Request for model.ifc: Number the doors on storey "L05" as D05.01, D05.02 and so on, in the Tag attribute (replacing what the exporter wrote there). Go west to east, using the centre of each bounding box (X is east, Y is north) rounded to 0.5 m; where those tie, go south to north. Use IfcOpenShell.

First a look at what the model holds.

```python
import ifcopenshell
import ifcopenshell.util.element
import ifcopenshell.util.placement

model = ifcopenshell.open("model.ifc")
print(model.schema)
storey = next(s for s in model.by_type("IfcBuildingStorey") if s.Name == "L05")
doors = [e for e in ifcopenshell.util.element.get_decomposition(storey) if e.is_a("IfcDoor")]
for e in sorted(doors, key=lambda e: e.id()):
    origin = ifcopenshell.util.placement.get_local_placement(e.ObjectPlacement)[:3, 3]
    print(e.id(), e.Tag, e.Name, origin.round(2) + 0.0, sep=" | ")
```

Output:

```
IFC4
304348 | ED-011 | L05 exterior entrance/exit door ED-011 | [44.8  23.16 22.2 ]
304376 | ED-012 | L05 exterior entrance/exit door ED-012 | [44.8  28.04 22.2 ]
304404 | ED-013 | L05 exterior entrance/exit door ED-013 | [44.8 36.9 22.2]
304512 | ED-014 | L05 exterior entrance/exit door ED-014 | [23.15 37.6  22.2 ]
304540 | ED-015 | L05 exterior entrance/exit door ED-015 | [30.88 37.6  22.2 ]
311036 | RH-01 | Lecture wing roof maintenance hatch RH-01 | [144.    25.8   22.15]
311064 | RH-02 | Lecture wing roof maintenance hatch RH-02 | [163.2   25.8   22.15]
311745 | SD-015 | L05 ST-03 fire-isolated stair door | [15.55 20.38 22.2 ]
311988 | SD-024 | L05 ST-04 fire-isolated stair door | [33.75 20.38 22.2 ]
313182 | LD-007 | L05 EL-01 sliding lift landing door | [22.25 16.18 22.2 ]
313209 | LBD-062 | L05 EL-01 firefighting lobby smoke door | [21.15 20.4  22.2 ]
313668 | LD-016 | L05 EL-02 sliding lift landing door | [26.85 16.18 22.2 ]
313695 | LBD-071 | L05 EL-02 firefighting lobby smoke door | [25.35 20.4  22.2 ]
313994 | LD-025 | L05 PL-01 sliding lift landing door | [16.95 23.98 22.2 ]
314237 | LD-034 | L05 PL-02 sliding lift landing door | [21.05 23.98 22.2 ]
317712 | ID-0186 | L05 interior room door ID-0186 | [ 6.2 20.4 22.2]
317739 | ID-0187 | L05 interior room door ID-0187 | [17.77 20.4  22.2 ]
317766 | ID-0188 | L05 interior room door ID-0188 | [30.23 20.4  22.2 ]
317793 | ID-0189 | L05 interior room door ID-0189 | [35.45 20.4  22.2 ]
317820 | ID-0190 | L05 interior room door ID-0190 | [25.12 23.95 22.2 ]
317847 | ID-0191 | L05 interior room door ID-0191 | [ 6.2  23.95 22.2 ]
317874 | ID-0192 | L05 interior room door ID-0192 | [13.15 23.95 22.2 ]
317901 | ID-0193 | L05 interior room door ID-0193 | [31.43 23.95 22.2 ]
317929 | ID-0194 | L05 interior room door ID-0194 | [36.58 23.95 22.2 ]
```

```python
import ifcopenshell
import ifcopenshell.geom
import ifcopenshell.util.element
import ifcopenshell.util.shape

model = ifcopenshell.open("model.ifc")
settings = ifcopenshell.geom.settings()
settings.set("use-world-coords", True)


def centre(element):
    shape = ifcopenshell.geom.create_shape(settings, element)
    return ifcopenshell.util.shape.get_bbox_centroid(shape.geometry)


storey = next(s for s in model.by_type("IfcBuildingStorey") if s.Name == "L05")
doors = [e for e in ifcopenshell.util.element.get_decomposition(storey) if e.is_a("IfcDoor")]

# Insertion points can sit at a corner or the storey origin, so sort by the geometry (in metres).
centres = {e: centre(e) for e in doors}
doors.sort(key=lambda e: (round(centres[e][0] / 0.5), centres[e][1]))

for i, e in enumerate(doors, start=1):
    number = f"D05.{i:02d}"
    e.Tag = number
    print(e.id(), number)

model.write("model_v2.ifc")
```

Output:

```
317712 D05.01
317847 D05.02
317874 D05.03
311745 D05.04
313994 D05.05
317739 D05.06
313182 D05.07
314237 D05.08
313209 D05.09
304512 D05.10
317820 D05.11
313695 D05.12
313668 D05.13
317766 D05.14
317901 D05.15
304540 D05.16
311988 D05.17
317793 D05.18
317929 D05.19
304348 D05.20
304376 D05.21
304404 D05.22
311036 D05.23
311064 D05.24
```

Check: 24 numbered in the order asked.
